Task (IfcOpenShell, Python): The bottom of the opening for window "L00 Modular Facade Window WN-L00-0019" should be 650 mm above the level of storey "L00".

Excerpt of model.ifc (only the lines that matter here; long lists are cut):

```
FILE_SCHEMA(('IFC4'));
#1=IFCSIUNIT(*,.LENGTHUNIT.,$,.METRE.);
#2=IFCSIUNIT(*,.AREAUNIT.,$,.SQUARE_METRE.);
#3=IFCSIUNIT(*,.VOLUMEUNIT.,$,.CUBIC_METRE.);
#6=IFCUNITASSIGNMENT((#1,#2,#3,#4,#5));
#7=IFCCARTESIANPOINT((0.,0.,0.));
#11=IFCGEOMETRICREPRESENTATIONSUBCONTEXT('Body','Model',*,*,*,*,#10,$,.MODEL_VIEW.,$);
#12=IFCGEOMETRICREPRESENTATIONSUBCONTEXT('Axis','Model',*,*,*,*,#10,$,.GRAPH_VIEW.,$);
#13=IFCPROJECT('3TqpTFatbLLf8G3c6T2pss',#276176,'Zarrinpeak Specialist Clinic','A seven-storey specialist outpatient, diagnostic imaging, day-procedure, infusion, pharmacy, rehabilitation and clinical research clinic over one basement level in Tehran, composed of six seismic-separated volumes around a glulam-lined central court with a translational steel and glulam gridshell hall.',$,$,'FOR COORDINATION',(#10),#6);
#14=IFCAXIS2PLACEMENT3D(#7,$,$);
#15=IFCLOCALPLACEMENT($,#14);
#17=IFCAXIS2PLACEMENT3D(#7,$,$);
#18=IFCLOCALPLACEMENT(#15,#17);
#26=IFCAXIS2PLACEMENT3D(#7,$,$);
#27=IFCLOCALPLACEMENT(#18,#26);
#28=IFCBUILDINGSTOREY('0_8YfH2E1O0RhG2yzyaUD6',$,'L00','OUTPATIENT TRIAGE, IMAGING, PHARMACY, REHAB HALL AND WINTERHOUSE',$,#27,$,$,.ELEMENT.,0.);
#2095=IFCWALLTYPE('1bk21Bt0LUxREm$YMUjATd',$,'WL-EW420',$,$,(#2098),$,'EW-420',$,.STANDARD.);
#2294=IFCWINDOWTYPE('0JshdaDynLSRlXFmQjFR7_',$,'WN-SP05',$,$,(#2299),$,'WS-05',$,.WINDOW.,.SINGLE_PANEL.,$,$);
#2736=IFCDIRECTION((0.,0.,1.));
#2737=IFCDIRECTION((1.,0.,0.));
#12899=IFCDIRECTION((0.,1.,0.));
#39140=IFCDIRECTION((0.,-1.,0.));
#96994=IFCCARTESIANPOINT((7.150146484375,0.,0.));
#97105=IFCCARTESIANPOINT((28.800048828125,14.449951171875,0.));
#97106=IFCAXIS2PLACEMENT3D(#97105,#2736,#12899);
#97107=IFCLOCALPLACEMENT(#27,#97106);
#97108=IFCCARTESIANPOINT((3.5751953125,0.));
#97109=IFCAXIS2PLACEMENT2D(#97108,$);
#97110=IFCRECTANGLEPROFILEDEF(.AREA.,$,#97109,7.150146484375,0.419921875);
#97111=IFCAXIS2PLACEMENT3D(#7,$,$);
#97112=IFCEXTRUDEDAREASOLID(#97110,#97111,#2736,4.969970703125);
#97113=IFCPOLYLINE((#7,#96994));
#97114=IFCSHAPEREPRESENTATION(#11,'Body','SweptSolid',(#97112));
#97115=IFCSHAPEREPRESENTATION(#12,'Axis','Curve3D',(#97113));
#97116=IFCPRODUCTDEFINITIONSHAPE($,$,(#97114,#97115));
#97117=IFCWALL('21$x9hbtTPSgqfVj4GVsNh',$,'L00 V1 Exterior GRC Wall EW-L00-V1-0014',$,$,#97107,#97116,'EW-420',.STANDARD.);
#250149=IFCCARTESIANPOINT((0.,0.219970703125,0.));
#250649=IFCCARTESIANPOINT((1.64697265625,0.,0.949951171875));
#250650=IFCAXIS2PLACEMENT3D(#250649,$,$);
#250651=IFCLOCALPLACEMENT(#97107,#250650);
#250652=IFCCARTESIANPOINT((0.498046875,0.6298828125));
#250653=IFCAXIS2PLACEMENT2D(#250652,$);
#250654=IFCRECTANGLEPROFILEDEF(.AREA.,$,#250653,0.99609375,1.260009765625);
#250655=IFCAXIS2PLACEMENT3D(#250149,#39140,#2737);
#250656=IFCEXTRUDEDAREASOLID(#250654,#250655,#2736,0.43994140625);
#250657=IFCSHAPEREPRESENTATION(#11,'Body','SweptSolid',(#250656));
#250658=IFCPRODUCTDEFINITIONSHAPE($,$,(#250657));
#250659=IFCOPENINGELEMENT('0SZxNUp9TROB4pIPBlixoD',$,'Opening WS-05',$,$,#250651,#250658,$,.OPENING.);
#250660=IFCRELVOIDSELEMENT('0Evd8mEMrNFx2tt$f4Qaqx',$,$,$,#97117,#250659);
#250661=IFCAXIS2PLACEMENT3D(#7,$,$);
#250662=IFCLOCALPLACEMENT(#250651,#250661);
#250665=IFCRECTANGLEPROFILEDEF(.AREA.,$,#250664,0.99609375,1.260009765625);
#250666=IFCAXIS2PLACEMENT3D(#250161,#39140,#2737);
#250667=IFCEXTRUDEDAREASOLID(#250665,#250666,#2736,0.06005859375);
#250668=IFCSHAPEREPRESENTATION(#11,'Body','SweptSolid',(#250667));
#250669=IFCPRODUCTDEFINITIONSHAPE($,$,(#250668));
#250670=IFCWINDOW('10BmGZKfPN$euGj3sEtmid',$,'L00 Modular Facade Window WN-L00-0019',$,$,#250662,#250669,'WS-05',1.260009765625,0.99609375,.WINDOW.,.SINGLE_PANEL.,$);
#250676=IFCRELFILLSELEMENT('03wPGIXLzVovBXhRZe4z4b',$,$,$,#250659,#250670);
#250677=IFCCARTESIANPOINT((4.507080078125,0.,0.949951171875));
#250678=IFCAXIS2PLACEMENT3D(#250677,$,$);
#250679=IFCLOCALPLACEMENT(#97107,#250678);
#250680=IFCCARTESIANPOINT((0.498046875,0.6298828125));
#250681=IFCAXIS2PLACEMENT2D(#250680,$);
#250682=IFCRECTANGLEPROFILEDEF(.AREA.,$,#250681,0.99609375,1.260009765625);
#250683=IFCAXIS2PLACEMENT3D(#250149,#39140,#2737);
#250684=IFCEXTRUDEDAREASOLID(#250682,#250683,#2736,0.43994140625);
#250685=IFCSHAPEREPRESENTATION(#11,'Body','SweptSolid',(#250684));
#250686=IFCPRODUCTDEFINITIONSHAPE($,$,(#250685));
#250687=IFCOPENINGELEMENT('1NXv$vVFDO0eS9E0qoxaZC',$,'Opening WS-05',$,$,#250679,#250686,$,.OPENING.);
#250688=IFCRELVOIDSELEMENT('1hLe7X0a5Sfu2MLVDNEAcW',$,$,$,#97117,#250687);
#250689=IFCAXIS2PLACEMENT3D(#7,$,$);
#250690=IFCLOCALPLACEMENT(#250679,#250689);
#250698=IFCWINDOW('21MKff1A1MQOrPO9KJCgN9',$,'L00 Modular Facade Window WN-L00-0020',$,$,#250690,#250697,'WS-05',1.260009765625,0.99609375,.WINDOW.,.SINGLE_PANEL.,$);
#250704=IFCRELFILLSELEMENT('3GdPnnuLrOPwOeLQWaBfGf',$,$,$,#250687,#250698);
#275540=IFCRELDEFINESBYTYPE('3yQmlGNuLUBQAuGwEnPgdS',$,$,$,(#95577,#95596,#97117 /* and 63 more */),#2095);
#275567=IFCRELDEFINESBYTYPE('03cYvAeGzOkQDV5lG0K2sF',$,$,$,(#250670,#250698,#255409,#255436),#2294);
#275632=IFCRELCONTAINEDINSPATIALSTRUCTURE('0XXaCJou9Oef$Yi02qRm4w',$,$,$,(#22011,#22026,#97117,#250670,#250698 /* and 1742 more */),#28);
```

```python
import numpy as np
import ifcopenshell
import ifcopenshell.api.geometry
import ifcopenshell.geom
import ifcopenshell.util.element
import ifcopenshell.util.placement
import ifcopenshell.util.shape
import ifcopenshell.util.unit

model = ifcopenshell.open("model.ifc")
unit_scale = ifcopenshell.util.unit.calculate_unit_scale(model)

window = model.by_guid("10BmGZKfPN$euGj3sEtmid")
opening = window.FillsVoids[0].RelatingOpeningElement
storey = ifcopenshell.util.element.get_container(window, ifc_class="IfcBuildingStorey")
level = ifcopenshell.util.placement.get_local_placement(storey.ObjectPlacement)[2, 3]

# The opening's origin need not be at the sill, so measure its lowest point.
shape = ifcopenshell.geom.create_shape(ifcopenshell.geom.settings(), opening)
bottom = ifcopenshell.util.shape.get_shape_bottom_elevation(shape, shape.geometry) / unit_scale
dz = level + 0.65 - bottom

shift = np.array([0.0, 0.0, dz])
# The window is placed relative to its opening, so it follows when the opening moves.
matrix = ifcopenshell.util.placement.get_local_placement(opening.ObjectPlacement)
matrix[:3, 3] += shift
ifcopenshell.api.geometry.edit_object_placement(
    model, product=opening, matrix=matrix, is_si=False, should_transform_children=True
)

print(f"moved by {dz * unit_scale:+.3f} m")

model.write("model_v2.ifc")
```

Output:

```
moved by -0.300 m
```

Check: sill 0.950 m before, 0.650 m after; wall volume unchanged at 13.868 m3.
